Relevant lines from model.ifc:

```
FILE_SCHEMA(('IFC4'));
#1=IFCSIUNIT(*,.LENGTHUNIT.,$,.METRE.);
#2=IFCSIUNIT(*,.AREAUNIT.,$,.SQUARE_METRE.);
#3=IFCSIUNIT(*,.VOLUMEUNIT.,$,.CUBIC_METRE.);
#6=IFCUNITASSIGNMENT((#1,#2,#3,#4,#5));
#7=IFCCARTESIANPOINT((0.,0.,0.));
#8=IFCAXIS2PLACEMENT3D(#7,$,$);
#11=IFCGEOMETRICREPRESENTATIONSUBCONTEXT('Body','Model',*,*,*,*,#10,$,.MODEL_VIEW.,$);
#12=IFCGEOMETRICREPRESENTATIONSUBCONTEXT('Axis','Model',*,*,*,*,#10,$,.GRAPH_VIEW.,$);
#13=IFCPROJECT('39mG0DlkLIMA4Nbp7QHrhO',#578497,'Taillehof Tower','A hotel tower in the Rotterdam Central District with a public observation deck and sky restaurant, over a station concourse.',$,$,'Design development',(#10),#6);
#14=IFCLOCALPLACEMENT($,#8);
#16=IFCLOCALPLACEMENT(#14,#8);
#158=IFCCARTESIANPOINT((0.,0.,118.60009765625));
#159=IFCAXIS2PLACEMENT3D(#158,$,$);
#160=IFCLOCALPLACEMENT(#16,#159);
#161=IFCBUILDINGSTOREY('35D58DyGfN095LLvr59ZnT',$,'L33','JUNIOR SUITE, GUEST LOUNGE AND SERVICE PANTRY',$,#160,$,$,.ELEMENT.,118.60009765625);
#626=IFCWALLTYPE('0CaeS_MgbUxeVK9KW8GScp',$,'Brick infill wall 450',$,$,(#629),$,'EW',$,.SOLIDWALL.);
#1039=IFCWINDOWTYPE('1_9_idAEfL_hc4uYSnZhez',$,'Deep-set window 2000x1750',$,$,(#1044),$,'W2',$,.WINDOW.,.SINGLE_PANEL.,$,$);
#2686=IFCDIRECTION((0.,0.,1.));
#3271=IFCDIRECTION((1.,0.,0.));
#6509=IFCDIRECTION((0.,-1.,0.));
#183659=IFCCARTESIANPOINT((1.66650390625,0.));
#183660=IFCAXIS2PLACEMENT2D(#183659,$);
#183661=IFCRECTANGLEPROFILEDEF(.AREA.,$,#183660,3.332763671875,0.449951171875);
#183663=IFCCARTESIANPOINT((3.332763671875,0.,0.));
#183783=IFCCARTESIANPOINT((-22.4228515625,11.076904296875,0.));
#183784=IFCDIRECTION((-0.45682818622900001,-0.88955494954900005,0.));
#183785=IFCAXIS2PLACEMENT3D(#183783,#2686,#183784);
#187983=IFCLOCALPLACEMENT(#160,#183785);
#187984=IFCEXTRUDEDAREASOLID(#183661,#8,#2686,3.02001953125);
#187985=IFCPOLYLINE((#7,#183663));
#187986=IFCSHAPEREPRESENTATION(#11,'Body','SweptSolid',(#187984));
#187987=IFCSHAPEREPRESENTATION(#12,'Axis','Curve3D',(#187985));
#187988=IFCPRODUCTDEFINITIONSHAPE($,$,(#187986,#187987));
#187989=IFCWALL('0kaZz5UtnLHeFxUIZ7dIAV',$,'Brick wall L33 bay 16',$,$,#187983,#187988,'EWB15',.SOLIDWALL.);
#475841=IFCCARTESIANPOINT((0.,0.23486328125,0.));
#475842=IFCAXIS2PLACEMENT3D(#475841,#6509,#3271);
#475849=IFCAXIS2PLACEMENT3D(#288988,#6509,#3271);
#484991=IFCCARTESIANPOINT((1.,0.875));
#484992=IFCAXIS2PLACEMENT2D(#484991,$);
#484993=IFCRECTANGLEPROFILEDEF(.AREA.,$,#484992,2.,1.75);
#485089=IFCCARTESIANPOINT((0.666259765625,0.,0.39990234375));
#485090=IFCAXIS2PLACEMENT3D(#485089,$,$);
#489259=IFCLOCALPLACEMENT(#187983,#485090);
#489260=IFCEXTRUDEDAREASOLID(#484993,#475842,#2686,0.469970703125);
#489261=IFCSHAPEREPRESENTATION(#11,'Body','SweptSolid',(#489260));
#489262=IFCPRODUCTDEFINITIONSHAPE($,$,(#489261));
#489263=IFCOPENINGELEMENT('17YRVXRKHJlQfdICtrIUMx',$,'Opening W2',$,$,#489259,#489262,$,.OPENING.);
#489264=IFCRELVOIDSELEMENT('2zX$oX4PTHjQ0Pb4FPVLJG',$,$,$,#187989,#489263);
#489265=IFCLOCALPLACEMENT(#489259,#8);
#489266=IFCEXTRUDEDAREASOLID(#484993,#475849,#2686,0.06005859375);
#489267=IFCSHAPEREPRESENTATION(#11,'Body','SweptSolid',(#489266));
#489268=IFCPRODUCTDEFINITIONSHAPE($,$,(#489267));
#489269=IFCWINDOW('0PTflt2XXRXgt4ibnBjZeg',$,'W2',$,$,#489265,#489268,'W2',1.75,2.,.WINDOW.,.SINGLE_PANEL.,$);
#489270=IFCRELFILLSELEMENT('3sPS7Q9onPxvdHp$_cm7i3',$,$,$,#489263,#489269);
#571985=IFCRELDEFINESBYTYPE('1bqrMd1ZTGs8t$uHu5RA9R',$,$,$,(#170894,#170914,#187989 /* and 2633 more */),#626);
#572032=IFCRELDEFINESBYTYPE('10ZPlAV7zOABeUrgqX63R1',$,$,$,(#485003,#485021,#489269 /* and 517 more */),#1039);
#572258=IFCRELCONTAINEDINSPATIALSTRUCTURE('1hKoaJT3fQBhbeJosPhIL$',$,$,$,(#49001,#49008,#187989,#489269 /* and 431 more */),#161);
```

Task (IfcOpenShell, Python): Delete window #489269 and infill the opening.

```python
import ifcopenshell
import ifcopenshell.api.feature
import ifcopenshell.api.root
import ifcopenshell.geom
import ifcopenshell.util.shape

model = ifcopenshell.open("model.ifc")
settings = ifcopenshell.geom.settings()


def volume(element):
    """Net volume in cubic metres, openings subtracted."""
    shape = ifcopenshell.geom.create_shape(settings, element)
    return ifcopenshell.util.shape.get_volume(shape.geometry)


window = model.by_guid("0PTflt2XXRXgt4ibnBjZeg")
opening = window.FillsVoids[0].RelatingOpeningElement
wall = opening.VoidsElements[0].RelatingBuildingElement
before = volume(wall)

ifcopenshell.api.root.remove_product(model, product=window)
ifcopenshell.api.feature.remove_feature(model, feature=opening)

after = volume(wall)

print(f"wall volume {before:.3f} -> {after:.3f} m3")

model.write("model_updated.ifc")
```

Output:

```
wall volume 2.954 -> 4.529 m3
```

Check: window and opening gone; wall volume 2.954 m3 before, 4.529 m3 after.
